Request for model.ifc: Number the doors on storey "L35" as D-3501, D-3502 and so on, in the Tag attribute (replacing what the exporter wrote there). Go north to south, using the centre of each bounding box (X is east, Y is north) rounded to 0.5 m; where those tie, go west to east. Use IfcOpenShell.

First a look at what the model holds.

```python
import ifcopenshell
import ifcopenshell.util.element
import ifcopenshell.util.placement

model = ifcopenshell.open("model.ifc")
print(model.schema)
storey = next(s for s in model.by_type("IfcBuildingStorey") if s.Name == "L35")
doors = [e for e in ifcopenshell.util.element.get_decomposition(storey) if e.is_a("IfcDoor")]
for e in sorted(doors, key=lambda e: e.id()):
    origin = ifcopenshell.util.placement.get_local_placement(e.ObjectPlacement)[:3, 3]
    print(e.id(), e.Tag, e.Name, origin.round(2) + 0.0, sep=" | ")
```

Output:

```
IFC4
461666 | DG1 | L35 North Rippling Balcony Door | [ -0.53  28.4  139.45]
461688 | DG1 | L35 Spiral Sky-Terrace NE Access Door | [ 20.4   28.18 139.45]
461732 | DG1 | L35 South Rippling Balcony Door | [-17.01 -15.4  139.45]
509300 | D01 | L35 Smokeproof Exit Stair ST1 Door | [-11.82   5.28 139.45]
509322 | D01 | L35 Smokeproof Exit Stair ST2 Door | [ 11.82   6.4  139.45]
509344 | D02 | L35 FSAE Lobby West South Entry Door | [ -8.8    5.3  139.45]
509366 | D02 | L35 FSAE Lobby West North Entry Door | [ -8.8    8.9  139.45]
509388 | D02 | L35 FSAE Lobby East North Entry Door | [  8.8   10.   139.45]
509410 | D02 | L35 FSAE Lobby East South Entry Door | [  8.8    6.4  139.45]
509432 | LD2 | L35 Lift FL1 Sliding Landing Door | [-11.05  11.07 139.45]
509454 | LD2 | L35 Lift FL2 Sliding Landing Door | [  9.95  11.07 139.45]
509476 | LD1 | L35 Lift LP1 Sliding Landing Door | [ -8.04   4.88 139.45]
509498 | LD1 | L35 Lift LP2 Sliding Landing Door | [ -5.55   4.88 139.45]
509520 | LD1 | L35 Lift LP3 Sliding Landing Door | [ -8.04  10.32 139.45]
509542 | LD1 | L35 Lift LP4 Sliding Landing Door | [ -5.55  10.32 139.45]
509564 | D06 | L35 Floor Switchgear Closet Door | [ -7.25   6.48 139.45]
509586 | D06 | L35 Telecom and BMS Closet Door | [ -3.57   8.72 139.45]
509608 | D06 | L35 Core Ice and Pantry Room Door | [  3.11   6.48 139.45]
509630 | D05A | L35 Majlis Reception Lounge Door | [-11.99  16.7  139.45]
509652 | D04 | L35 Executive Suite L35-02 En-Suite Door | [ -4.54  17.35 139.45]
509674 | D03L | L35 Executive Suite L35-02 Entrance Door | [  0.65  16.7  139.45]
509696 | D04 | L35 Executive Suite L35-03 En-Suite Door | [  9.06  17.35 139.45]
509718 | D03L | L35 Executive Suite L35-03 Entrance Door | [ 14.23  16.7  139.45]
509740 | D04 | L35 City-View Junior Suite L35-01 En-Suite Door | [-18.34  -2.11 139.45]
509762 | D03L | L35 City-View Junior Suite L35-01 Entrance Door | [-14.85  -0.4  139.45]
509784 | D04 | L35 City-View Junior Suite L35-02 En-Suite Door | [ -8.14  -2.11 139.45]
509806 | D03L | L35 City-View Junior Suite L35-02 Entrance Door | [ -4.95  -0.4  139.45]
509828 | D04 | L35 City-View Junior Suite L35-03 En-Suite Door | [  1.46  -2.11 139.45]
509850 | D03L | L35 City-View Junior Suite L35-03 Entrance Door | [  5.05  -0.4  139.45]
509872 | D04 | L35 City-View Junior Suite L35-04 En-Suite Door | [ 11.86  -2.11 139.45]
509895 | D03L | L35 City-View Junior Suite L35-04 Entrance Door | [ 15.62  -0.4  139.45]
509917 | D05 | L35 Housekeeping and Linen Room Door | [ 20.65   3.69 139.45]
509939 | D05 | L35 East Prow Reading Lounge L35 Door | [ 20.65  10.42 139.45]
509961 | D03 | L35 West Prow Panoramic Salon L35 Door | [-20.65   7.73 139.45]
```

```python
import ifcopenshell
import ifcopenshell.geom
import ifcopenshell.util.element
import ifcopenshell.util.shape

model = ifcopenshell.open("model.ifc")
settings = ifcopenshell.geom.settings()
settings.set("use-world-coords", True)


def centre(element):
    shape = ifcopenshell.geom.create_shape(settings, element)
    return ifcopenshell.util.shape.get_bbox_centroid(shape.geometry)


storey = next(s for s in model.by_type("IfcBuildingStorey") if s.Name == "L35")
doors = [e for e in ifcopenshell.util.element.get_decomposition(storey) if e.is_a("IfcDoor")]

# Insertion points can sit at a corner or the storey origin, so sort by the geometry (in metres).
centres = {e: centre(e) for e in doors}
doors.sort(key=lambda e: (-round(centres[e][1] / 0.5), centres[e][0]))

for i, e in enumerate(doors, start=1):
    number = f"D-35{i:02d}"
    e.Tag = number
    print(e.id(), number)

model.write("model-out.ifc")
```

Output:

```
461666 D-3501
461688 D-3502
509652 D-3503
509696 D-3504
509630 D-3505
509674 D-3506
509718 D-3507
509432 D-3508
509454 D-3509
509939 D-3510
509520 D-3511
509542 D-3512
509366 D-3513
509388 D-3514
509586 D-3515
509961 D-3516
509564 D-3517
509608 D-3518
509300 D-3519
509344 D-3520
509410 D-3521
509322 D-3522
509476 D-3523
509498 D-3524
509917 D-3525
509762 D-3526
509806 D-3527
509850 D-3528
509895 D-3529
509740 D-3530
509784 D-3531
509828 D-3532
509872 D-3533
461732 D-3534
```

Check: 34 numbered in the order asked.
